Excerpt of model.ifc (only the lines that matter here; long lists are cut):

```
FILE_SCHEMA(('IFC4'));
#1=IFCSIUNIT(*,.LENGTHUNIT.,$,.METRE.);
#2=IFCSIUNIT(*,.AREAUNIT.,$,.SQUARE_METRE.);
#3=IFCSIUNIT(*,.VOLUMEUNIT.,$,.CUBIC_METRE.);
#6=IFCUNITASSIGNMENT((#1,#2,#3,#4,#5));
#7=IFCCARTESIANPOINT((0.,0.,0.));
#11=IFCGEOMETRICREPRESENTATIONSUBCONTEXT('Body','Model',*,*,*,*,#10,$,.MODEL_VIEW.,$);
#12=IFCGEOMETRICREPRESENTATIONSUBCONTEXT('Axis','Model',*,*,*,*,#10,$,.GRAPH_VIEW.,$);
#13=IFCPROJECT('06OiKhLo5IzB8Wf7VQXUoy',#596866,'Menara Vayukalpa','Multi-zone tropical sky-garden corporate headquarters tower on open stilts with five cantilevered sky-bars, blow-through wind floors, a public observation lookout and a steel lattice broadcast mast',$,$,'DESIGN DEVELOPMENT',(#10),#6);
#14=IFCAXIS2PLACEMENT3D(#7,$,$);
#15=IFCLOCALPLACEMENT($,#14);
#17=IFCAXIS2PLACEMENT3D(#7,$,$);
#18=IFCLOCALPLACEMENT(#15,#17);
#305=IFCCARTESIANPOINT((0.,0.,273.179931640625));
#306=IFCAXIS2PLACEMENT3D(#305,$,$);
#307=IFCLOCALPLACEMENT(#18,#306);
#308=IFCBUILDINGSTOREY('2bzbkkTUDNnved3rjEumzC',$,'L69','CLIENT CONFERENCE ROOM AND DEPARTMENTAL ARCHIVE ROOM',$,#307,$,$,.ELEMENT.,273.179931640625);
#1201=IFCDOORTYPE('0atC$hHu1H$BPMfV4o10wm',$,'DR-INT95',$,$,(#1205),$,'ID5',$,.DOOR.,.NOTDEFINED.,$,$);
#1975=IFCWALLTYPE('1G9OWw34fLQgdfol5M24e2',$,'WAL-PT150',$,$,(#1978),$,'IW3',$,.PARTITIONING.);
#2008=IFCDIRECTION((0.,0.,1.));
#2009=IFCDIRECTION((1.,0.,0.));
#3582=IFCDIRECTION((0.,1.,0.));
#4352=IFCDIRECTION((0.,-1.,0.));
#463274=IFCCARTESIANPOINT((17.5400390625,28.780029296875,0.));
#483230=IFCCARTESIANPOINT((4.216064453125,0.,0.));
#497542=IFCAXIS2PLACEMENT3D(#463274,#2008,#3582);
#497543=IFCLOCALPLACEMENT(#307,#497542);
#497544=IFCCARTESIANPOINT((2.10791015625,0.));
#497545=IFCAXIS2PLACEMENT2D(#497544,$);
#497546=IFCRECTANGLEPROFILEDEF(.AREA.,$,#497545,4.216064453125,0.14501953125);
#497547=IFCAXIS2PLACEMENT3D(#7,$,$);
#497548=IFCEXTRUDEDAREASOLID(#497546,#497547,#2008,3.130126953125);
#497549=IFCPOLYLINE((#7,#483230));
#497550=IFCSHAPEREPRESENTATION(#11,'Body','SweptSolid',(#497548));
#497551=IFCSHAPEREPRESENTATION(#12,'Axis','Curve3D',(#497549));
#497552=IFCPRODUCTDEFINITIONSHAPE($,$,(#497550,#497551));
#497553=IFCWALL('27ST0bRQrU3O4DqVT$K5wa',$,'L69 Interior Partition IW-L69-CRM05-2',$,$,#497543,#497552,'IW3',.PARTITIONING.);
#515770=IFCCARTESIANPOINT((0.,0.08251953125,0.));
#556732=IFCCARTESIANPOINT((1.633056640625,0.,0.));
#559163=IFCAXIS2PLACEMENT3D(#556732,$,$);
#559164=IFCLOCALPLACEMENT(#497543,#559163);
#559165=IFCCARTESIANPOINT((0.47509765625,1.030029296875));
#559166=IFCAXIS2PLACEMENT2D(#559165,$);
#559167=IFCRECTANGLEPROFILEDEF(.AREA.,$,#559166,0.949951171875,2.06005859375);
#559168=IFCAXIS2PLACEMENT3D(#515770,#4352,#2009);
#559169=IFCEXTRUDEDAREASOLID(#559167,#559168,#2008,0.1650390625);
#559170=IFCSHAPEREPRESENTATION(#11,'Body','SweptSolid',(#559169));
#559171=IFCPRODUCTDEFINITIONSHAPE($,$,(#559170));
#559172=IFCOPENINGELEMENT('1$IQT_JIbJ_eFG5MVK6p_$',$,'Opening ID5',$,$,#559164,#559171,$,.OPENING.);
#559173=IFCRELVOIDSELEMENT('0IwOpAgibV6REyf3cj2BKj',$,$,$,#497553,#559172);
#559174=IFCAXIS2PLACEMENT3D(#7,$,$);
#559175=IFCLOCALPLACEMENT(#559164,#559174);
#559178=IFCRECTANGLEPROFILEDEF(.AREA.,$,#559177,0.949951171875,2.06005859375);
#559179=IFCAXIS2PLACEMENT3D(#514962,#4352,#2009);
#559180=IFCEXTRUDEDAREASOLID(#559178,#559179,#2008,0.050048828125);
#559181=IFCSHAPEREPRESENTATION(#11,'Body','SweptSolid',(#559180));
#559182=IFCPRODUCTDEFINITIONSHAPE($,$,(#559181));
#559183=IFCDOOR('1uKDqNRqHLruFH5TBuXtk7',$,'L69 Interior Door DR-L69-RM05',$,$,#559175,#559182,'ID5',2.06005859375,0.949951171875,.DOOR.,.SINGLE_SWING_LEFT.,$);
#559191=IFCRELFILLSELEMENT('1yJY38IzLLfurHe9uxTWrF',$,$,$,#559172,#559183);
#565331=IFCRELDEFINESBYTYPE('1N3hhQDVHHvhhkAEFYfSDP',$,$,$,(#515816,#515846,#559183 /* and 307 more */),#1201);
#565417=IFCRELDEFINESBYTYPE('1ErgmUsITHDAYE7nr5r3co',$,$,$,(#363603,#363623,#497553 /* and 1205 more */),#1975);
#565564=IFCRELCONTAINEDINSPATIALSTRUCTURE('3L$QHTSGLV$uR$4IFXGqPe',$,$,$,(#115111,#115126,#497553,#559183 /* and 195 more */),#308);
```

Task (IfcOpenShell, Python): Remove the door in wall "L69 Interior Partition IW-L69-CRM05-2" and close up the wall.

```python
import ifcopenshell
import ifcopenshell.api.feature
import ifcopenshell.api.root
import ifcopenshell.geom
import ifcopenshell.util.shape

model = ifcopenshell.open("model.ifc")
settings = ifcopenshell.geom.settings()


def volume(element):
    """Net volume in cubic metres, openings subtracted."""
    shape = ifcopenshell.geom.create_shape(settings, element)
    return ifcopenshell.util.shape.get_volume(shape.geometry)


door = model.by_guid("1uKDqNRqHLruFH5TBuXtk7")
opening = door.FillsVoids[0].RelatingOpeningElement
wall = opening.VoidsElements[0].RelatingBuildingElement
before = volume(wall)

ifcopenshell.api.root.remove_product(model, product=door)
ifcopenshell.api.feature.remove_feature(model, feature=opening)

after = volume(wall)

print(f"wall volume {before:.3f} -> {after:.3f} m3")

model.write("model_rev.ifc")
```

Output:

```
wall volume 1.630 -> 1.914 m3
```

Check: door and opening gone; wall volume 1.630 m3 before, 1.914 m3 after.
